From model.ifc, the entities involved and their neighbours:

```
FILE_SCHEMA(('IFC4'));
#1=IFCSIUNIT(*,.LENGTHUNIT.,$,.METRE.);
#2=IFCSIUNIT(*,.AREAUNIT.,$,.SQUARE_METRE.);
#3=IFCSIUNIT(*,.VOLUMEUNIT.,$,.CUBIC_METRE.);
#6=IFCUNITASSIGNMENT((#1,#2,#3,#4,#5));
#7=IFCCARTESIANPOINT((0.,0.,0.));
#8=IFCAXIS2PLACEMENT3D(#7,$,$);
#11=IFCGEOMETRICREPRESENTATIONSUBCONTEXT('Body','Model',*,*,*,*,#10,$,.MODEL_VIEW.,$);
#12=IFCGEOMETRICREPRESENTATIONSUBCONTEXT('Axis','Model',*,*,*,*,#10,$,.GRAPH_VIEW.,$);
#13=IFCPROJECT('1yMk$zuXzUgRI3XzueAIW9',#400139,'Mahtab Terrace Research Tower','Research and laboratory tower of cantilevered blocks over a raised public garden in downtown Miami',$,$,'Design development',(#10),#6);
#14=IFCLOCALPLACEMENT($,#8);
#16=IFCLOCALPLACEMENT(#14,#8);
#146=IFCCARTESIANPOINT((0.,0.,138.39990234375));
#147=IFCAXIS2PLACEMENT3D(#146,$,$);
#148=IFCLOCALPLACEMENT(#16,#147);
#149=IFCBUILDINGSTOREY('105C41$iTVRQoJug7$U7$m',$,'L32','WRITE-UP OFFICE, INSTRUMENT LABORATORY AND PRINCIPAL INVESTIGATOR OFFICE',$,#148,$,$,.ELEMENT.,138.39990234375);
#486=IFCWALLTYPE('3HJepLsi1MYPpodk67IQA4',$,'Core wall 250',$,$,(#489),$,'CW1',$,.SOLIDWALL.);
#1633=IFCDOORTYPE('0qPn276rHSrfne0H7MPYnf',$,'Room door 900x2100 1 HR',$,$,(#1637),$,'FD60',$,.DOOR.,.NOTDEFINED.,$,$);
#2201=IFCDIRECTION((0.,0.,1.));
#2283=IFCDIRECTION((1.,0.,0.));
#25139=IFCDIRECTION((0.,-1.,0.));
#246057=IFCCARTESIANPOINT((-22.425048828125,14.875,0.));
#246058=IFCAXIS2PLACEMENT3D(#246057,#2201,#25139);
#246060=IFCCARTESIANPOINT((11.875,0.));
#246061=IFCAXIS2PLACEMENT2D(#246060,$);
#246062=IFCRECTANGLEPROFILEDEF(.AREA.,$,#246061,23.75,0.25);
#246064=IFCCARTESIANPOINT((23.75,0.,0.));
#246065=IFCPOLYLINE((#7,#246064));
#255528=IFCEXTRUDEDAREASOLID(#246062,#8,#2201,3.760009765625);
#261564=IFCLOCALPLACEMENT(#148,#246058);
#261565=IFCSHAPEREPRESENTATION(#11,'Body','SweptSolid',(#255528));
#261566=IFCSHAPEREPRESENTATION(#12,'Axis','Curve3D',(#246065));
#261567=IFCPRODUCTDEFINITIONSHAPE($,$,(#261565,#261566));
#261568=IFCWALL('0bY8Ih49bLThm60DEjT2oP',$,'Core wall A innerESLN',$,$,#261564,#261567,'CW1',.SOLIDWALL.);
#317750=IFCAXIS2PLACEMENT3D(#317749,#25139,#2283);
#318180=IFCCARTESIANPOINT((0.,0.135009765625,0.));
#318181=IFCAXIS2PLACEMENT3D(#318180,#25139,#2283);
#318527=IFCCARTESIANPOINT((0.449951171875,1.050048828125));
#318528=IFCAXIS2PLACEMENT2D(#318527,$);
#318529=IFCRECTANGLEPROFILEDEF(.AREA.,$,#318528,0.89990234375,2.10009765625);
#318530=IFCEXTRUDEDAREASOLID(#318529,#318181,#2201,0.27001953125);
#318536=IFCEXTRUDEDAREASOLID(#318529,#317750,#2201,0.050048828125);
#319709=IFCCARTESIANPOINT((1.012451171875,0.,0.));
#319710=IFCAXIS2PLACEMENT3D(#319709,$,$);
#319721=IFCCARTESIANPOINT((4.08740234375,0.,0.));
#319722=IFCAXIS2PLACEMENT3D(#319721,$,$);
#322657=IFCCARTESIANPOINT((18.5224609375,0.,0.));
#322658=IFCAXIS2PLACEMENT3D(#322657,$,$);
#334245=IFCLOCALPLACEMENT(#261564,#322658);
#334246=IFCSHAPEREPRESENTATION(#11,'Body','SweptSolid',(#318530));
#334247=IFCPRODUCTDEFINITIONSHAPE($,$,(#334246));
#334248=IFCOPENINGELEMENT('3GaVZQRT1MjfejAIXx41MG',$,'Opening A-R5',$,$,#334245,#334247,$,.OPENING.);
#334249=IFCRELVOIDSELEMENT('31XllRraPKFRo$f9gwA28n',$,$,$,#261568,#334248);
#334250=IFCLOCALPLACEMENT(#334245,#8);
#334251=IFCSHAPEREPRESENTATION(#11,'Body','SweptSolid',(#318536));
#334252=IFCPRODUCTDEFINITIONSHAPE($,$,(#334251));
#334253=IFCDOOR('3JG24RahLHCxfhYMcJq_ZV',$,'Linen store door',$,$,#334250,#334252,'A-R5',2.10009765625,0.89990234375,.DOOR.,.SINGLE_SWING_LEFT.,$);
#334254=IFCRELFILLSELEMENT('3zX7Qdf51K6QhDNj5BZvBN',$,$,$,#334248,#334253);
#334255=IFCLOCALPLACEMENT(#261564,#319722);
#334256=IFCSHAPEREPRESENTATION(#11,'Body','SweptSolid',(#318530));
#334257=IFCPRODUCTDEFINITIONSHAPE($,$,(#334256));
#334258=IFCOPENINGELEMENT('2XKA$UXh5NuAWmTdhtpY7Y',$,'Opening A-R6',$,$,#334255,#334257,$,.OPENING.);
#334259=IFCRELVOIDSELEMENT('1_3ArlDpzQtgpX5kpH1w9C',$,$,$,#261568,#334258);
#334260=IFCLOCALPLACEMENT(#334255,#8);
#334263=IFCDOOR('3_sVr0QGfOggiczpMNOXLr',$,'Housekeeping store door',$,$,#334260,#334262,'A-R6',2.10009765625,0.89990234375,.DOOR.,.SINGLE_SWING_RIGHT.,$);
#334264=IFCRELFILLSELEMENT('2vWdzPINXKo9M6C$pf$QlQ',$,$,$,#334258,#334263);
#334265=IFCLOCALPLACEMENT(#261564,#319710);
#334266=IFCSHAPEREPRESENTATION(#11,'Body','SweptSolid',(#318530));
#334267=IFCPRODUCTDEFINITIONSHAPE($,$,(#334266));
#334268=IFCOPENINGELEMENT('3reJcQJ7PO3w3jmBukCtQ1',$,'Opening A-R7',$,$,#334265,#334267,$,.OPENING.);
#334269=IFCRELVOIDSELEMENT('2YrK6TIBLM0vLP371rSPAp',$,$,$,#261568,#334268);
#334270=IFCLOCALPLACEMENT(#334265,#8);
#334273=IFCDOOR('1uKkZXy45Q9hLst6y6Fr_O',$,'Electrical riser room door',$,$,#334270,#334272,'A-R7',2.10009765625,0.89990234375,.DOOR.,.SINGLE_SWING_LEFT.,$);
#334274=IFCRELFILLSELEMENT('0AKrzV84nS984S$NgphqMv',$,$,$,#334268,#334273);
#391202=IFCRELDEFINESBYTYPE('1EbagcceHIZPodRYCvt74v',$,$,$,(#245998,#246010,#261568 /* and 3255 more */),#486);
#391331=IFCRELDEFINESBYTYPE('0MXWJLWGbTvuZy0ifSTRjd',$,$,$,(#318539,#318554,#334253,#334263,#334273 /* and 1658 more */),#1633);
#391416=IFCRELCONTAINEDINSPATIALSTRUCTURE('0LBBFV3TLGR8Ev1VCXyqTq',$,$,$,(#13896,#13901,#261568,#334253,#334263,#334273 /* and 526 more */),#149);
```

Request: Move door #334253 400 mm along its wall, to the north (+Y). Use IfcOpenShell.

```python
import ifcopenshell
import ifcopenshell.api.geometry
import ifcopenshell.util.placement
import ifcopenshell.util.unit

model = ifcopenshell.open("model.ifc")
unit_scale = ifcopenshell.util.unit.calculate_unit_scale(model)

door = model.by_guid("3JG24RahLHCxfhYMcJq_ZV")
opening = door.FillsVoids[0].RelatingOpeningElement
wall = opening.VoidsElements[0].RelatingBuildingElement

wall_matrix = ifcopenshell.util.placement.get_local_placement(wall.ObjectPlacement)
shift = wall_matrix[:3, 0] * -0.4 / unit_scale
before = ifcopenshell.util.placement.get_local_placement(door.ObjectPlacement)[:3, 3].copy()

# The door is placed relative to its opening, so it follows when the opening moves.
matrix = ifcopenshell.util.placement.get_local_placement(opening.ObjectPlacement)
matrix[:3, 3] += shift
ifcopenshell.api.geometry.edit_object_placement(
    model, product=opening, matrix=matrix, is_si=False, should_transform_children=True
)

after = ifcopenshell.util.placement.get_local_placement(door.ObjectPlacement)[:3, 3]
print("door moved by", (after - before).round(3) + 0.0)

model.write("model_updated.ifc")
```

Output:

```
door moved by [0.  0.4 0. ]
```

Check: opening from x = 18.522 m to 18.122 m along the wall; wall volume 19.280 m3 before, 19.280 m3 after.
